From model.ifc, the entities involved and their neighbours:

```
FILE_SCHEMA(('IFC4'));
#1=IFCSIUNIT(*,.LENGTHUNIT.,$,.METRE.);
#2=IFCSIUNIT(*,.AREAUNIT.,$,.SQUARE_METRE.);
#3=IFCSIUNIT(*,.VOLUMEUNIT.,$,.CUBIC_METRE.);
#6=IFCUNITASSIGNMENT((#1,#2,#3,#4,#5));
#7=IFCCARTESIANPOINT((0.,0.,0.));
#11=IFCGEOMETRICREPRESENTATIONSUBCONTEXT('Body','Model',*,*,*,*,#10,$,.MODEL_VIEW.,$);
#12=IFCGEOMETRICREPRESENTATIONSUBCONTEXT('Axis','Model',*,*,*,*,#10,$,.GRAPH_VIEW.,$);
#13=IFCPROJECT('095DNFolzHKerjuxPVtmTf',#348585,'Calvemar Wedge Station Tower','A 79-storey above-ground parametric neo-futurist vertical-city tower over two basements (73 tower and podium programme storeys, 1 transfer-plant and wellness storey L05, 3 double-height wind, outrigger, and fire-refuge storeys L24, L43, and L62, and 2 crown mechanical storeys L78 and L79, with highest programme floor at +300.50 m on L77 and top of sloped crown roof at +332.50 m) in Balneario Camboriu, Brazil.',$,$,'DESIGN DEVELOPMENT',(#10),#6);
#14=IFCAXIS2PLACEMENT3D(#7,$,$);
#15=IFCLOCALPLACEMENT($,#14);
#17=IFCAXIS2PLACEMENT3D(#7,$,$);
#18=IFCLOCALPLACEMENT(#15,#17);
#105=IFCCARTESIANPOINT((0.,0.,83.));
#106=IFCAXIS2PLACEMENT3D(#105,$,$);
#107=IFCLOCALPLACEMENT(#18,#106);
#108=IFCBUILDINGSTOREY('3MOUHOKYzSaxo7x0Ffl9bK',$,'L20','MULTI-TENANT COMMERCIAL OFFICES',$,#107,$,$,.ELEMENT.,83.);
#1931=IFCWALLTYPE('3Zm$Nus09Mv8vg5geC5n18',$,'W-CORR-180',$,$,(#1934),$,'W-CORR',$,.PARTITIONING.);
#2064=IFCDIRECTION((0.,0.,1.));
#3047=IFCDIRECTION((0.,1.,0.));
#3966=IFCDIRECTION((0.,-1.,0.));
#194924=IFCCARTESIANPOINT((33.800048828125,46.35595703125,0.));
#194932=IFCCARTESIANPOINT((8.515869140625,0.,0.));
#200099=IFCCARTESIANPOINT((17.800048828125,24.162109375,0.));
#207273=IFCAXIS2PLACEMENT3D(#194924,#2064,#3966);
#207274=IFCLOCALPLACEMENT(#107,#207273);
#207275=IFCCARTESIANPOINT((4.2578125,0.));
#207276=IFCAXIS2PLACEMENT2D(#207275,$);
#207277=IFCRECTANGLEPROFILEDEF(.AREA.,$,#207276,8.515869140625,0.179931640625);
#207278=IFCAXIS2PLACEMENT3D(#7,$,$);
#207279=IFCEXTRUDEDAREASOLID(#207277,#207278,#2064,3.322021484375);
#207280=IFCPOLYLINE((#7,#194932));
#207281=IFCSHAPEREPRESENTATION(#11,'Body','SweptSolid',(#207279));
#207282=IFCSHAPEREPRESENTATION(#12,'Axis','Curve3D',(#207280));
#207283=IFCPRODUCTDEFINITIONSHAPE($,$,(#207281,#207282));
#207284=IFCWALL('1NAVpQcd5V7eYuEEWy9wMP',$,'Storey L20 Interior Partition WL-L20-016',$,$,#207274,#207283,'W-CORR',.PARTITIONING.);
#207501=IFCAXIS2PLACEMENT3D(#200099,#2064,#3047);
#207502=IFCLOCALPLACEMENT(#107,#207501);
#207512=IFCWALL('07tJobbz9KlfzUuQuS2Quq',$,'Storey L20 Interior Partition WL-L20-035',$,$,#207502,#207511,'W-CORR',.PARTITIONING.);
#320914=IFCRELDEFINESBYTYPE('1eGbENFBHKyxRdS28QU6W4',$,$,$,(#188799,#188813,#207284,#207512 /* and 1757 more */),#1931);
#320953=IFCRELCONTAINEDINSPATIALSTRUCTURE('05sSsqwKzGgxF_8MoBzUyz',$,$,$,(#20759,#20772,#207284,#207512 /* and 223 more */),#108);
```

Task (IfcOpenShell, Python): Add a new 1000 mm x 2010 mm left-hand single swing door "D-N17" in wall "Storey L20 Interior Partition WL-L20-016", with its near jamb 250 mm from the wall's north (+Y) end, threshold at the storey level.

```python
import numpy as np
import ifcopenshell
import ifcopenshell.api.feature
import ifcopenshell.api.geometry
import ifcopenshell.api.root
import ifcopenshell.api.spatial
import ifcopenshell.geom
import ifcopenshell.util.element
import ifcopenshell.util.placement
import ifcopenshell.util.representation
import ifcopenshell.util.shape
import ifcopenshell.util.unit

model = ifcopenshell.open("model.ifc")
unit_scale = ifcopenshell.util.unit.calculate_unit_scale(model)
settings = ifcopenshell.geom.settings()


def volume(element):
    """Net volume in cubic metres, openings subtracted."""
    shape = ifcopenshell.geom.create_shape(settings, element)
    return ifcopenshell.util.shape.get_volume(shape.geometry)


wall = model.by_guid("1NAVpQcd5V7eYuEEWy9wMP")
storey = ifcopenshell.util.element.get_container(wall, ifc_class="IfcBuildingStorey")
context = ifcopenshell.util.representation.get_context(model, "Model", "Body", "MODEL_VIEW")
before = volume(wall)

width, height, from_end, sill = 1, 2.01, 0.25, 0.0  # metres

# The wall runs along its own X axis, and the end named is its -X end.
wall_shape = ifcopenshell.geom.create_shape(settings, wall)
x, y, z = ifcopenshell.util.shape.get_vertices(wall_shape.geometry).T
start = x.min() + from_end
face, thickness = float(y.min()), float(y.max() - y.min())
wall_matrix = ifcopenshell.util.placement.get_local_placement(wall.ObjectPlacement)
level = ifcopenshell.util.placement.get_local_placement(storey.ObjectPlacement)[2, 3]


def in_wall(x, y):
    """Placement at x, y metres in the wall's axes, at sill height."""
    matrix = wall_matrix.copy()
    matrix[:, 3] = wall_matrix @ np.array([x / unit_scale, y / unit_scale, 0.0, 1.0])
    matrix[2, 3] = level + sill / unit_scale
    return matrix


# Opening: a box that overshoots both wall faces by 50 mm.
opening = ifcopenshell.api.root.create_entity(model, ifc_class="IfcOpeningElement", predefined_type="OPENING")
box = ifcopenshell.api.geometry.add_wall_representation(
    model, context=context, length=width, height=height, thickness=thickness + 0.1
)
ifcopenshell.api.geometry.assign_representation(model, product=opening, representation=box)
ifcopenshell.api.geometry.edit_object_placement(model, product=opening, matrix=in_wall(start, face - 0.05), is_si=False)
ifcopenshell.api.feature.add_feature(model, feature=opening, element=wall)

door = ifcopenshell.api.root.create_entity(model, ifc_class="IfcDoor", name="D-N17", predefined_type="DOOR")
door.OverallWidth, door.OverallHeight = width / unit_scale, height / unit_scale
door.OperationType = "SINGLE_SWING_LEFT"
body = ifcopenshell.api.geometry.add_door_representation(
    model,
    context=context,
    overall_width=door.OverallWidth,
    overall_height=door.OverallHeight,
    operation_type="SINGLE_SWING_LEFT",
    lining_properties={"LiningDepth": thickness / unit_scale, "ThresholdDepth": thickness / unit_scale},
)
ifcopenshell.api.geometry.assign_representation(model, product=door, representation=body)
ifcopenshell.api.spatial.assign_container(model, products=[door], relating_structure=storey)
ifcopenshell.api.feature.add_filling(model, opening=opening, element=door)

# The lining spans the wall, so the door starts at the wall face.
ifcopenshell.api.geometry.edit_object_placement(model, product=door, matrix=in_wall(start, face), is_si=False)

after = volume(wall)

print(f"wall volume {before:.3f} -> {after:.3f} m3")

model.write("model_edited.ifc")
```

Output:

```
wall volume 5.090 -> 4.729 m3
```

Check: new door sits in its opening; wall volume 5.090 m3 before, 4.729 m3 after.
